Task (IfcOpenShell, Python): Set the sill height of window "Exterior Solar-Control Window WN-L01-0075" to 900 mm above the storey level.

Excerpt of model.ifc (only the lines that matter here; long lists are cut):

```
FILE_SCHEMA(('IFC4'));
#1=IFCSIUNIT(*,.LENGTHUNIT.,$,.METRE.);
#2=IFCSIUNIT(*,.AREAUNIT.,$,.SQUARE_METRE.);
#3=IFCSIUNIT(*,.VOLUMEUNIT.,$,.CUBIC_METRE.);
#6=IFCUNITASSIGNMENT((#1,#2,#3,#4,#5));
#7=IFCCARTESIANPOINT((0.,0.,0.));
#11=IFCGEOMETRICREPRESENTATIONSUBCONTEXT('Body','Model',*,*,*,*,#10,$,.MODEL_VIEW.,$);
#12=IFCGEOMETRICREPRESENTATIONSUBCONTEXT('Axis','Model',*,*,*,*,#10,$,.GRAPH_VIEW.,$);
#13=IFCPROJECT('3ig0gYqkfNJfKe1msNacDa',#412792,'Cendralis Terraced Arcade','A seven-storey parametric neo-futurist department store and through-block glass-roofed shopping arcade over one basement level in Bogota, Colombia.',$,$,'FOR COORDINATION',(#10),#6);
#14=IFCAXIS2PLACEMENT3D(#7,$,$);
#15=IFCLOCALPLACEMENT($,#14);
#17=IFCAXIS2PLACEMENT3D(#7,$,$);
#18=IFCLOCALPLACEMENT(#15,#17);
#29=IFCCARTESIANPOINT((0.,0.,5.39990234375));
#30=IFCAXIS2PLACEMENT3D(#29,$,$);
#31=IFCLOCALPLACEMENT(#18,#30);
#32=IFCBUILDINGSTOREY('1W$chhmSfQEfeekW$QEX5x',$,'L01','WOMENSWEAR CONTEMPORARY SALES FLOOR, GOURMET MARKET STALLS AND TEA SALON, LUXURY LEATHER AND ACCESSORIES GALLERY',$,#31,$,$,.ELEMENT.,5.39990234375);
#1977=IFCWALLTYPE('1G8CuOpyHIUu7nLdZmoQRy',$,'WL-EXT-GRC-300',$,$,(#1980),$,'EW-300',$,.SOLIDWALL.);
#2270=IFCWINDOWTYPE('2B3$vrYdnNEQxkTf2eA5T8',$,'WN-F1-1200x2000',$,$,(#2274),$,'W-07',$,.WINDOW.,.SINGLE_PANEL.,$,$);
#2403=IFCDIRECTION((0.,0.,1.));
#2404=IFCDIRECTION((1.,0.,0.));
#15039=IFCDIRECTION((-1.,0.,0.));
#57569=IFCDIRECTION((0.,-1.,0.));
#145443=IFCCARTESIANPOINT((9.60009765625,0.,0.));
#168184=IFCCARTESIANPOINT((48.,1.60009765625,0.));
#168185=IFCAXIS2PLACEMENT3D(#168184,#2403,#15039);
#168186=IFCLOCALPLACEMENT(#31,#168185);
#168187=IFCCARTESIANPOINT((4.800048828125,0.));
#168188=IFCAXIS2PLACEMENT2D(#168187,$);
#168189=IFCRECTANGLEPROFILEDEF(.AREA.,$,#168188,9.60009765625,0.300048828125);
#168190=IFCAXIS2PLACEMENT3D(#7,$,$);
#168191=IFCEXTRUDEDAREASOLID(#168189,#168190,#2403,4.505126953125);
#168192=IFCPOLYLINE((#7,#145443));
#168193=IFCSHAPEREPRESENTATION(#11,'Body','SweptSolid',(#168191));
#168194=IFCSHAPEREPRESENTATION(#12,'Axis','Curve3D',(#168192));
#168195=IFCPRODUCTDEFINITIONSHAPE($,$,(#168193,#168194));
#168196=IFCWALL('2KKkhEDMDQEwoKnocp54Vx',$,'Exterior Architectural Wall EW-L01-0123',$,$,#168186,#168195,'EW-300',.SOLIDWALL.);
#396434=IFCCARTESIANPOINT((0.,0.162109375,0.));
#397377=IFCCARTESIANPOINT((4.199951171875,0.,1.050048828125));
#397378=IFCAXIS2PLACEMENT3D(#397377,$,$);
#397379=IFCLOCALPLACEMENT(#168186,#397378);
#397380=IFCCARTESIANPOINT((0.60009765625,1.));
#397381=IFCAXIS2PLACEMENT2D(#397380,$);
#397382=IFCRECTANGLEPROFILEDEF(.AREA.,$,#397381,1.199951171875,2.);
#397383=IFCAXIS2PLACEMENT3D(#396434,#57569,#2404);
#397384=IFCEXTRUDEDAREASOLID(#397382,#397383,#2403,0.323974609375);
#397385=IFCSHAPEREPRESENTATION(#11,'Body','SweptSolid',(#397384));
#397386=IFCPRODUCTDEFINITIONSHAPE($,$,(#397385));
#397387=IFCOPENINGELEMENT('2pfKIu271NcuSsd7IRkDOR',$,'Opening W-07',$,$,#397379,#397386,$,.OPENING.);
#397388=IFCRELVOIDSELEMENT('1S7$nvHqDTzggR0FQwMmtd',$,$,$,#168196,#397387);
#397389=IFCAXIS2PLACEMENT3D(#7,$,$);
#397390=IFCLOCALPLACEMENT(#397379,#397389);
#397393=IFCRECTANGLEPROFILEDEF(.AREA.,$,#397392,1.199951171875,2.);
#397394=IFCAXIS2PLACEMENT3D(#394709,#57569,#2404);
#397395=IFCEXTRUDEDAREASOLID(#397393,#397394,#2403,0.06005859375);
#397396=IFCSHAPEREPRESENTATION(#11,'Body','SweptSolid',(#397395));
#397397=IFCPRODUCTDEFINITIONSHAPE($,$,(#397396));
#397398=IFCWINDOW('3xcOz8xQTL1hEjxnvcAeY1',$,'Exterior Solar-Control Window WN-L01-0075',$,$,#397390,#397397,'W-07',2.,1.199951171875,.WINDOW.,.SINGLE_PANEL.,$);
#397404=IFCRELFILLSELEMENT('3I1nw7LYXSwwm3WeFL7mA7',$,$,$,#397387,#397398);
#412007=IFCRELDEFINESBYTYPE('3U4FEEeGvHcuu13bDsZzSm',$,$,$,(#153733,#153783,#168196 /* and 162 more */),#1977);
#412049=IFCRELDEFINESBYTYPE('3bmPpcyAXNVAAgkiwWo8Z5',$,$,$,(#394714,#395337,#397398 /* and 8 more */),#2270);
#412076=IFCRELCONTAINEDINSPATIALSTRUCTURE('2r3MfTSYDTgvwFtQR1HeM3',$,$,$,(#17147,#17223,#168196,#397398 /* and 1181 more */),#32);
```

```python
import numpy as np
import ifcopenshell
import ifcopenshell.api.geometry
import ifcopenshell.geom
import ifcopenshell.util.element
import ifcopenshell.util.placement
import ifcopenshell.util.shape
import ifcopenshell.util.unit

model = ifcopenshell.open("model.ifc")
unit_scale = ifcopenshell.util.unit.calculate_unit_scale(model)

window = model.by_guid("3xcOz8xQTL1hEjxnvcAeY1")
opening = window.FillsVoids[0].RelatingOpeningElement
storey = ifcopenshell.util.element.get_container(window, ifc_class="IfcBuildingStorey")
level = ifcopenshell.util.placement.get_local_placement(storey.ObjectPlacement)[2, 3]

# The opening's origin need not be at the sill, so measure its lowest point.
shape = ifcopenshell.geom.create_shape(ifcopenshell.geom.settings(), opening)
bottom = ifcopenshell.util.shape.get_shape_bottom_elevation(shape, shape.geometry) / unit_scale
dz = level + 0.9 - bottom

shift = np.array([0.0, 0.0, dz])
# The window is placed relative to its opening, so it follows when the opening moves.
matrix = ifcopenshell.util.placement.get_local_placement(opening.ObjectPlacement)
matrix[:3, 3] += shift
ifcopenshell.api.geometry.edit_object_placement(
    model, product=opening, matrix=matrix, is_si=False, should_transform_children=True
)

print(f"moved by {dz * unit_scale:+.3f} m")

model.write("model-out.ifc")
```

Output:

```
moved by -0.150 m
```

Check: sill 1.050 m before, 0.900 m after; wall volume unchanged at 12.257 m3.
